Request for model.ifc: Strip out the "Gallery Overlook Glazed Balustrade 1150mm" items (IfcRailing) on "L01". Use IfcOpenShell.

First a look at what the model holds.

```python
import ifcopenshell
import ifcopenshell.util.element

model = ifcopenshell.open("model.ifc")
print(model.schema)
storey = next(s for s in model.by_type("IfcBuildingStorey") if s.Name == "L01")
railings = [e for e in ifcopenshell.util.element.get_decomposition(storey) if e.is_a("IfcRailing")]
seen = {}
for e in railings:
    element_type = ifcopenshell.util.element.get_type(e)
    name = element_type.Name if element_type not in (None, e) else None
    seen[name] = seen.get(name, 0) + 1
for name, count in sorted(seen.items(), key=str):
    print(count, "x", name)
```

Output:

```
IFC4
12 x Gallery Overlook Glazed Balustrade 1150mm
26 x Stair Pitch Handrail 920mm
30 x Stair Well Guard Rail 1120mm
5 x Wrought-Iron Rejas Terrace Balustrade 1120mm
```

```python
import ifcopenshell
import ifcopenshell.api.root
import ifcopenshell.util.element

model = ifcopenshell.open("model.ifc")

storey = next(s for s in model.by_type("IfcBuildingStorey") if s.Name == "L01")
railings = [e for e in ifcopenshell.util.element.get_decomposition(storey) if e.is_a("IfcRailing")]
targets = [e for e in railings if (t := ifcopenshell.util.element.get_type(e)) not in (None, e) and t.Name == "Gallery Overlook Glazed Balustrade 1150mm"]

for e in targets:
    ifcopenshell.api.root.remove_product(model, product=e)
print(len(targets), "removed")

model.write("model_updated.ifc")
```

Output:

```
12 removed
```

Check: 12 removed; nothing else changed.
